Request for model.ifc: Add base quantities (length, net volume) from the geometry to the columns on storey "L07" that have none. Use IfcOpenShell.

First a look at what the model holds.

```python
import ifcopenshell
import ifcopenshell.util.element
import ifcopenshell.util.unit

model = ifcopenshell.open("model.ifc")
print(model.schema)
for unit_type in ("LENGTHUNIT", "AREAUNIT", "VOLUMEUNIT"):
    print(unit_type, ifcopenshell.util.unit.calculate_unit_scale(model, unit_type))
storey = next(s for s in model.by_type("IfcBuildingStorey") if s.Name == "L07")
columns = [e for e in ifcopenshell.util.element.get_decomposition(storey) if e.is_a("IfcColumn")]
for e in sorted(columns, key=lambda e: e.id()):
    print(e.id(), e.is_a(), e.Name, list(ifcopenshell.util.element.get_psets(e, qtos_only=True)), sep=" | ")
```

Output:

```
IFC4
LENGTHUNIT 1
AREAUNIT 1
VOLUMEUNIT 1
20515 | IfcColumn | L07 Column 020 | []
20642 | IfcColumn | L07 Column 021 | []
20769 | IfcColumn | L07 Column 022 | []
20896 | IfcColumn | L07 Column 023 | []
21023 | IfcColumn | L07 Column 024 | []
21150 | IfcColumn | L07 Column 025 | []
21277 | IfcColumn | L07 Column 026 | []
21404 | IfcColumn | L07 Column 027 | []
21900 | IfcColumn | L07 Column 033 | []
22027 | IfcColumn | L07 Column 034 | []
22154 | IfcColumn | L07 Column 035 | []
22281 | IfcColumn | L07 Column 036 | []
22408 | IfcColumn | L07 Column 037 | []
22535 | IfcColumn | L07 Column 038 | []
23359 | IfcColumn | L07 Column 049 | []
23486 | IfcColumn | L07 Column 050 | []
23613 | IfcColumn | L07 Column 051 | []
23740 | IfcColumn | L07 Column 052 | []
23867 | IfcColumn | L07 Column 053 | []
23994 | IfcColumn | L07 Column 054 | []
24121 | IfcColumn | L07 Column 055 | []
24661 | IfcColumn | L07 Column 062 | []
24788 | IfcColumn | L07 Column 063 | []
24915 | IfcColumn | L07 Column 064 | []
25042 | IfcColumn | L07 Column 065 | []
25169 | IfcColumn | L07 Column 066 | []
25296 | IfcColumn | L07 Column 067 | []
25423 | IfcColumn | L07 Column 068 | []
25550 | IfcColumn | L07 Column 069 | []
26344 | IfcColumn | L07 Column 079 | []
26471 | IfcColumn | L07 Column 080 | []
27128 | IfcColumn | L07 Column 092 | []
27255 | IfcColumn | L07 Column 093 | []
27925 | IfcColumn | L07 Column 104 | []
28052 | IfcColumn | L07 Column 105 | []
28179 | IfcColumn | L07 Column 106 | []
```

```python
import ifcopenshell
import ifcopenshell.api.pset
import ifcopenshell.geom
import ifcopenshell.util.element
import ifcopenshell.util.shape
import ifcopenshell.util.unit

model = ifcopenshell.open("model.ifc")
unit_scale = ifcopenshell.util.unit.calculate_unit_scale(model)
volume_scale = ifcopenshell.util.unit.calculate_unit_scale(model, "VOLUMEUNIT")
settings = ifcopenshell.geom.settings()

storey = next(s for s in model.by_type("IfcBuildingStorey") if s.Name == "L07")
columns = [e for e in ifcopenshell.util.element.get_decomposition(storey) if e.is_a("IfcColumn")]

for e in sorted(columns, key=lambda e: e.id()):
    if ifcopenshell.util.element.get_psets(e, qtos_only=True, should_inherit=False):
        continue
    # Geometry comes back in metres, in the element's own axes.
    shape = ifcopenshell.geom.create_shape(settings, e)
    values = {
        "Length": ifcopenshell.util.shape.get_z(shape.geometry) / unit_scale,
        "NetVolume": ifcopenshell.util.shape.get_volume(shape.geometry) / volume_scale,
    }
    qto = ifcopenshell.api.pset.add_qto(model, product=e, name="Qto_ColumnBaseQuantities")
    ifcopenshell.api.pset.edit_qto(model, qto=qto, properties=values)
    print(e.id(), {k: round(v, 3) for k, v in values.items()})

model.write("model-out.ifc")
```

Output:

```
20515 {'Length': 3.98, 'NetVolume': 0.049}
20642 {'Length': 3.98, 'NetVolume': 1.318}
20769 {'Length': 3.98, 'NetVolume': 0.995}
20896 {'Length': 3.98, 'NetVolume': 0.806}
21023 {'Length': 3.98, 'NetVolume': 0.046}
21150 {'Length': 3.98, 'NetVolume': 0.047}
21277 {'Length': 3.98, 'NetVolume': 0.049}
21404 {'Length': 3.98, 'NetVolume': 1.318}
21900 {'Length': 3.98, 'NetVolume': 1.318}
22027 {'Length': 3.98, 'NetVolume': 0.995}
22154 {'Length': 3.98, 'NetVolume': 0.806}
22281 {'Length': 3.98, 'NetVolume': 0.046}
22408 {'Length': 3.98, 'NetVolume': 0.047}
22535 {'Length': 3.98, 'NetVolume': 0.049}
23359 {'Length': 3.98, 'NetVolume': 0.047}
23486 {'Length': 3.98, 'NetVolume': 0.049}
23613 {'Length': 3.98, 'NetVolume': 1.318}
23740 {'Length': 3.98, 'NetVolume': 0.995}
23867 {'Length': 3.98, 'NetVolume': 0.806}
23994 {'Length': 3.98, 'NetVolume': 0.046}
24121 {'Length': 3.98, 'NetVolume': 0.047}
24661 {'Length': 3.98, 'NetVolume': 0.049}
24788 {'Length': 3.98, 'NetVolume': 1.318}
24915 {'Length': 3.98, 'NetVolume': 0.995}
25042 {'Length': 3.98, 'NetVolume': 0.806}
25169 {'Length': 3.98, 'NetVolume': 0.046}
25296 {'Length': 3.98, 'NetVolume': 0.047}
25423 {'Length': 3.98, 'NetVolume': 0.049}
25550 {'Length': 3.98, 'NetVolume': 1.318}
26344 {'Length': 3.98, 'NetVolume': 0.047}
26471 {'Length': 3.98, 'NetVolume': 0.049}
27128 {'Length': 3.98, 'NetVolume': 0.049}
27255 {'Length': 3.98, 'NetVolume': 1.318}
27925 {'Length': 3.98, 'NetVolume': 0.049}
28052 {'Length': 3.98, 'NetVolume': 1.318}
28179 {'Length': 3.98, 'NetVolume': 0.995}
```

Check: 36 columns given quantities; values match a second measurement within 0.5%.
